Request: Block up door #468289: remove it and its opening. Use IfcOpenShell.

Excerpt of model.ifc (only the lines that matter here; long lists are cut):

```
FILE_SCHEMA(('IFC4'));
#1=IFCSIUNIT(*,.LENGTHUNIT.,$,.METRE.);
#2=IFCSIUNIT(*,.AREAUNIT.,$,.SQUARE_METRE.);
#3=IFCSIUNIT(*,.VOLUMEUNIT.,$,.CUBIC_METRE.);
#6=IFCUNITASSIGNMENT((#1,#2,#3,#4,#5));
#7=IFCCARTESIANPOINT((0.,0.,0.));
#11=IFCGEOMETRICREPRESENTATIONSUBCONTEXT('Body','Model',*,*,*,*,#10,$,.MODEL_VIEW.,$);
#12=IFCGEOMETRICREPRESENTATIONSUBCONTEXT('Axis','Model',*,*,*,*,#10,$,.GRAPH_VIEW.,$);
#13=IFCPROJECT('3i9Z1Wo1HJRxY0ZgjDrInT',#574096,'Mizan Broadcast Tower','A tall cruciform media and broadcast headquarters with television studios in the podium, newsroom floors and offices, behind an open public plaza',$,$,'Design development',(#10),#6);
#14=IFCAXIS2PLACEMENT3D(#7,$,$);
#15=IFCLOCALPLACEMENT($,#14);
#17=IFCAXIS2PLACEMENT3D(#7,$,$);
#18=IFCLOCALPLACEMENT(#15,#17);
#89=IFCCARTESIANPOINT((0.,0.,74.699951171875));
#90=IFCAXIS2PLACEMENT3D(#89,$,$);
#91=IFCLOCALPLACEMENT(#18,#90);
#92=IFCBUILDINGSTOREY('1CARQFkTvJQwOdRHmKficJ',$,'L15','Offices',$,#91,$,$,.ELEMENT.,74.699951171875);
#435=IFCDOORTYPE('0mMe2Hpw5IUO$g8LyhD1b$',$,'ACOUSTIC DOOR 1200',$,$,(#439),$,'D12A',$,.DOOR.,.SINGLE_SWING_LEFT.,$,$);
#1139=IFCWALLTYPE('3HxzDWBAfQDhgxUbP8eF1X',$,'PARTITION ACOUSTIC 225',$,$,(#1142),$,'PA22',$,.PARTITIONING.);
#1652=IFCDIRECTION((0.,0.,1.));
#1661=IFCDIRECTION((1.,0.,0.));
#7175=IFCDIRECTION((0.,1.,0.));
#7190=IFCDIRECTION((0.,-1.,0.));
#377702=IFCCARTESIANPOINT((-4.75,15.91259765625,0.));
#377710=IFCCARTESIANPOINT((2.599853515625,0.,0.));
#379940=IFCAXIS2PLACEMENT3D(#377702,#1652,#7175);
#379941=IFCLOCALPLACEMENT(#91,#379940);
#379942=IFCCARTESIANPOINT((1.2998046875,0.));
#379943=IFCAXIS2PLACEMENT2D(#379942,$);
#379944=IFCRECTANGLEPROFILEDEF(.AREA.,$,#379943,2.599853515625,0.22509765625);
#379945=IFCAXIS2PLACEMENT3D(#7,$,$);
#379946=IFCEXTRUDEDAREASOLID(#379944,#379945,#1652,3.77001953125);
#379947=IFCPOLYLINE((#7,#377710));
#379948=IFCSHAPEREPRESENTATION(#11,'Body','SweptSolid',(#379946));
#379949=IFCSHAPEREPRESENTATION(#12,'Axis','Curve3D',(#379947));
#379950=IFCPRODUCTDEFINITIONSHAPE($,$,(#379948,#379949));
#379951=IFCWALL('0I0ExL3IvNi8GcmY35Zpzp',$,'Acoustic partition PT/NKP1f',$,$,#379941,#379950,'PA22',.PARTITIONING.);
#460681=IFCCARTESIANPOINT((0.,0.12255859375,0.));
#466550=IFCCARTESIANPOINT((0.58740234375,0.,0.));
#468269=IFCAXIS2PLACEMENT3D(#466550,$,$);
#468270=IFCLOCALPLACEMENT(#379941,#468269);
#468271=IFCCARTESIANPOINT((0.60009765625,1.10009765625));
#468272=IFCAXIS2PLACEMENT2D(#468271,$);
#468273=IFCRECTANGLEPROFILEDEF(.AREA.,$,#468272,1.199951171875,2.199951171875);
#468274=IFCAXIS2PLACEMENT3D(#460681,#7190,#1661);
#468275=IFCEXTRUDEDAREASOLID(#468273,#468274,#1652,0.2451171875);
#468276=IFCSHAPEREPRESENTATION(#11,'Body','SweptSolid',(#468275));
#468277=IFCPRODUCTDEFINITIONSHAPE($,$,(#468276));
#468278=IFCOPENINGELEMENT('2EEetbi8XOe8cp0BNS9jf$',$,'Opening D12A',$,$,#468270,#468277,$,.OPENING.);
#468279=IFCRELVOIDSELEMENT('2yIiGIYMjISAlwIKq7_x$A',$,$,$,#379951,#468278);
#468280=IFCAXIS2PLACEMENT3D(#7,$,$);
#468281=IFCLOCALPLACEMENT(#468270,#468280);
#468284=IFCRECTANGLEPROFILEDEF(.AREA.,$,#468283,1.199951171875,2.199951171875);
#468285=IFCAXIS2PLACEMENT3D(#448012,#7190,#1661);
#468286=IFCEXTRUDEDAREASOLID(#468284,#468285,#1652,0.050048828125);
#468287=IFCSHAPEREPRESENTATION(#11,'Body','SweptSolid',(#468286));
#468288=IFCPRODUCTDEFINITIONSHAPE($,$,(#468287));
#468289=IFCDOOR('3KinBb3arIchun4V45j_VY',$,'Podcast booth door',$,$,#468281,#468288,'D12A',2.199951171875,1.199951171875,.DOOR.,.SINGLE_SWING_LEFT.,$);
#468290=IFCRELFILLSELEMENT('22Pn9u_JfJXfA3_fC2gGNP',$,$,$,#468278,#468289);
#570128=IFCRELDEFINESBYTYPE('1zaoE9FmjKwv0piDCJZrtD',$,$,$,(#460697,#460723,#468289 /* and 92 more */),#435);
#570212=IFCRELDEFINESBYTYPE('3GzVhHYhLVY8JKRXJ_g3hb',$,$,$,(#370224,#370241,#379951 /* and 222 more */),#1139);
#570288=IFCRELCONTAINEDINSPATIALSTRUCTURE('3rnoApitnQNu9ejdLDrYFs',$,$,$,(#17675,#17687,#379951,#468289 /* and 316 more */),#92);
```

```python
import ifcopenshell
import ifcopenshell.api.feature
import ifcopenshell.api.root
import ifcopenshell.geom
import ifcopenshell.util.shape

model = ifcopenshell.open("model.ifc")
settings = ifcopenshell.geom.settings()


def volume(element):
    """Net volume in cubic metres, openings subtracted."""
    shape = ifcopenshell.geom.create_shape(settings, element)
    return ifcopenshell.util.shape.get_volume(shape.geometry)


door = model.by_guid("3KinBb3arIchun4V45j_VY")
opening = door.FillsVoids[0].RelatingOpeningElement
wall = opening.VoidsElements[0].RelatingBuildingElement
before = volume(wall)

ifcopenshell.api.root.remove_product(model, product=door)
ifcopenshell.api.feature.remove_feature(model, feature=opening)

after = volume(wall)

print(f"wall volume {before:.3f} -> {after:.3f} m3")

model.write("model_rev.ifc")
```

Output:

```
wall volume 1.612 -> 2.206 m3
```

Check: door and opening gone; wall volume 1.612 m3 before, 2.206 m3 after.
